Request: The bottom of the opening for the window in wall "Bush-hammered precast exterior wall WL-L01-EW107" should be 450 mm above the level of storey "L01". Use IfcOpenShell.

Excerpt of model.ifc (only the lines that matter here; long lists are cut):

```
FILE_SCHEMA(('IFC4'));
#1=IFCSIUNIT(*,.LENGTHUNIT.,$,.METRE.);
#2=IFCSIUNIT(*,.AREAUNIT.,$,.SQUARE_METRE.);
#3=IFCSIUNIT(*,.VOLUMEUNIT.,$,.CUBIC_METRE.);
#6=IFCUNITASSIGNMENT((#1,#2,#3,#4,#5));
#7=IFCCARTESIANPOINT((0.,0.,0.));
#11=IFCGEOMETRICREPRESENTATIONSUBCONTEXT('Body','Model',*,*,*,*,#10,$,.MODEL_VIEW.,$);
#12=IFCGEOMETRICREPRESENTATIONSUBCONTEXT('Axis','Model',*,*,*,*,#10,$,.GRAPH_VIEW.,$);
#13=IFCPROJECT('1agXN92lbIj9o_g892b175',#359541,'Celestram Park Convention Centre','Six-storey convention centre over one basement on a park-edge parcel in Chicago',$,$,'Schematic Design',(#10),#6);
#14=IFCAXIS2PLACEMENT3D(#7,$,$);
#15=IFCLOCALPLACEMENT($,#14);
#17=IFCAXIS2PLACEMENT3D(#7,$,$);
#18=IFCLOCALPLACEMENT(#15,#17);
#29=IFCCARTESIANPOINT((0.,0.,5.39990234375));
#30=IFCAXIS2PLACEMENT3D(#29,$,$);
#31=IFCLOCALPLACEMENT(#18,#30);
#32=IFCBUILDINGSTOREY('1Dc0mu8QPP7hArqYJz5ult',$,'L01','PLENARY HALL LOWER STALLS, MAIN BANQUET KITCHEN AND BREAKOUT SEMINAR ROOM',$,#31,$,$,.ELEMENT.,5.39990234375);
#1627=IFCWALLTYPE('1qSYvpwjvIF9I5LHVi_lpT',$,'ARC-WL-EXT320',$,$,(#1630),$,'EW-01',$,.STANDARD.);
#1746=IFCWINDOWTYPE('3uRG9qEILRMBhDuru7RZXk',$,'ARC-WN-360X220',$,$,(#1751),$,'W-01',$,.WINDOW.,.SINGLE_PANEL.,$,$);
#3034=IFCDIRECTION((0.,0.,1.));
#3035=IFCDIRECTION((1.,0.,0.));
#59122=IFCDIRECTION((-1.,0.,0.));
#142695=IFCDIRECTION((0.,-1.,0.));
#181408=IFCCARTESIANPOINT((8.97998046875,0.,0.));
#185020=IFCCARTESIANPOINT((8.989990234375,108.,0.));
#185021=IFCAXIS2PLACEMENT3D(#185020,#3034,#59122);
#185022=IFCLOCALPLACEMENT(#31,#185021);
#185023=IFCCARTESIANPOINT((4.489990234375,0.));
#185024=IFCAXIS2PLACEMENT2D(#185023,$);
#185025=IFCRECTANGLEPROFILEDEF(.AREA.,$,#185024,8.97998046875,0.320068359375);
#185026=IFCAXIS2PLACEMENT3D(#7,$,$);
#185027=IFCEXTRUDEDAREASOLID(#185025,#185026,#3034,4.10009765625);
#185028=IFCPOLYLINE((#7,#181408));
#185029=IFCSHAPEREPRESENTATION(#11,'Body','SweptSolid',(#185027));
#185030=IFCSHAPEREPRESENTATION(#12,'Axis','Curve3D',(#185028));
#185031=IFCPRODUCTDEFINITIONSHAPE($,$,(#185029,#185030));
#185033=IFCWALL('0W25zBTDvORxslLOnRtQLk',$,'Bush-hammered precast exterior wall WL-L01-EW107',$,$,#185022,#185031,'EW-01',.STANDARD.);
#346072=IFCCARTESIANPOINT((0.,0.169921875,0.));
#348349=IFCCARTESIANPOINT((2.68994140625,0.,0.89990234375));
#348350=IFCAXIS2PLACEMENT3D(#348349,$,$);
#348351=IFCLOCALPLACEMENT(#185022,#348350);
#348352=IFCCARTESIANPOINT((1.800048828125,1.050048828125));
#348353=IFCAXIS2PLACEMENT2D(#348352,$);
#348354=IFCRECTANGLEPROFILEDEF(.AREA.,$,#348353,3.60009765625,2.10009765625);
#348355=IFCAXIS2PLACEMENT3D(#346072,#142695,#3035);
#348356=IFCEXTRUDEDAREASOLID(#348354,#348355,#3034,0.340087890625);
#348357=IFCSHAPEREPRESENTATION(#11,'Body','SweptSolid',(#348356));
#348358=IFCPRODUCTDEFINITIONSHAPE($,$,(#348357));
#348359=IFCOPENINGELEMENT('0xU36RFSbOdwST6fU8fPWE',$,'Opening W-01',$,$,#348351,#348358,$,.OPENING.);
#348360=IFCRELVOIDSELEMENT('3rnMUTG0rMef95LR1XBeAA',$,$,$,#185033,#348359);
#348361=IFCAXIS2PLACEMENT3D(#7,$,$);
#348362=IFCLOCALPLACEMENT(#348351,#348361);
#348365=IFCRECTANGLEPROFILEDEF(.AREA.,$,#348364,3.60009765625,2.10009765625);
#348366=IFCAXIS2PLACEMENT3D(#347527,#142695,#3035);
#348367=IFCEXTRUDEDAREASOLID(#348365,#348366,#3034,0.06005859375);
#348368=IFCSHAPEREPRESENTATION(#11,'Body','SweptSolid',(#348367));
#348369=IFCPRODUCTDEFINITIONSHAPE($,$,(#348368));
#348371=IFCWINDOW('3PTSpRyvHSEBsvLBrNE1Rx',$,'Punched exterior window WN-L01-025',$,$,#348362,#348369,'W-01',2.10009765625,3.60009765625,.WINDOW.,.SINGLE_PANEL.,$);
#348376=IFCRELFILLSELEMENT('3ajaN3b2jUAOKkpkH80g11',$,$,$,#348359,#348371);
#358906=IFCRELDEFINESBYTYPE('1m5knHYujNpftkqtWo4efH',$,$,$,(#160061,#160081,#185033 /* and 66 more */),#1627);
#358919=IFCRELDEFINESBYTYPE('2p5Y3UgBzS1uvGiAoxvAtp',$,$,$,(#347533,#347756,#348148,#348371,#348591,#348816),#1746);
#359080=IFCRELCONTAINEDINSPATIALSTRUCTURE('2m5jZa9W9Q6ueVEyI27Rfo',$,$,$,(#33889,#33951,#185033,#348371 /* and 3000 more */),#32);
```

```python
import numpy as np
import ifcopenshell
import ifcopenshell.api.geometry
import ifcopenshell.geom
import ifcopenshell.util.element
import ifcopenshell.util.placement
import ifcopenshell.util.shape
import ifcopenshell.util.unit

model = ifcopenshell.open("model.ifc")
unit_scale = ifcopenshell.util.unit.calculate_unit_scale(model)

window = model.by_guid("3PTSpRyvHSEBsvLBrNE1Rx")
opening = window.FillsVoids[0].RelatingOpeningElement
storey = ifcopenshell.util.element.get_container(window, ifc_class="IfcBuildingStorey")
level = ifcopenshell.util.placement.get_local_placement(storey.ObjectPlacement)[2, 3]

# The opening's origin need not be at the sill, so measure its lowest point.
shape = ifcopenshell.geom.create_shape(ifcopenshell.geom.settings(), opening)
bottom = ifcopenshell.util.shape.get_shape_bottom_elevation(shape, shape.geometry) / unit_scale
dz = level + 0.45 - bottom

shift = np.array([0.0, 0.0, dz])
# The window is placed relative to its opening, so it follows when the opening moves.
matrix = ifcopenshell.util.placement.get_local_placement(opening.ObjectPlacement)
matrix[:3, 3] += shift
ifcopenshell.api.geometry.edit_object_placement(
    model, product=opening, matrix=matrix, is_si=False, should_transform_children=True
)

print(f"moved by {dz * unit_scale:+.3f} m")

model.write("model-out.ifc")
```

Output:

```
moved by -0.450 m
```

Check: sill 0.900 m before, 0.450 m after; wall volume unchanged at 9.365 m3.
